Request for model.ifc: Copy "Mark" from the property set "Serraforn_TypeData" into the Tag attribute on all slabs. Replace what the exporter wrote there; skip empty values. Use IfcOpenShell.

First a look at what the model holds.

```python
import ifcopenshell
import ifcopenshell.util.element

model = ifcopenshell.open("model.ifc")
print(model.schema)
slabs = model.by_type("IfcSlab")
print(len(slabs), "slabs")
for e in slabs[:8]:
    source = ifcopenshell.util.element.get_pset(e, "Serraforn_TypeData", "Mark")
    target = e.Tag
    print(e.id(), repr(source), repr(target), sep=" | ")
```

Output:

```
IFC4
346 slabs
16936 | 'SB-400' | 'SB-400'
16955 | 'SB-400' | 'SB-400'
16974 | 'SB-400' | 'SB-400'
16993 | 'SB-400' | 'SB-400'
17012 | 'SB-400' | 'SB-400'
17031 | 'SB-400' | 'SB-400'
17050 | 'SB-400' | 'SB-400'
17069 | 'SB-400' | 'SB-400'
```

```python
import ifcopenshell
import ifcopenshell.util.element

model = ifcopenshell.open("model.ifc")

count = 0
for e in model.by_type("IfcSlab"):
    value = ifcopenshell.util.element.get_pset(e, "Serraforn_TypeData", "Mark")
    current = e.Tag
    if not value or not value.strip() or current == value:
        continue
    e.Tag = value
    count += 1

print(count, "slabs updated")

model.write("model_updated.ifc")
```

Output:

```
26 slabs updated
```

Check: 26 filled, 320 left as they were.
